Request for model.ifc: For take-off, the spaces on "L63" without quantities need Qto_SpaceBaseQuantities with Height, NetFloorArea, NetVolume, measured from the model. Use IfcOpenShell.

First a look at what the model holds.

```python
import ifcopenshell
import ifcopenshell.util.element
import ifcopenshell.util.unit

model = ifcopenshell.open("model.ifc")
print(model.schema)
for unit_type in ("LENGTHUNIT", "AREAUNIT", "VOLUMEUNIT"):
    print(unit_type, ifcopenshell.util.unit.calculate_unit_scale(model, unit_type))
storey = next(s for s in model.by_type("IfcBuildingStorey") if s.Name == "L63")
spaces = [e for e in ifcopenshell.util.element.get_decomposition(storey) if e.is_a("IfcSpace")]
for e in sorted(spaces, key=lambda e: e.id()):
    print(e.id(), e.is_a(), e.Name, list(ifcopenshell.util.element.get_psets(e, qtos_only=True)), sep=" | ")
```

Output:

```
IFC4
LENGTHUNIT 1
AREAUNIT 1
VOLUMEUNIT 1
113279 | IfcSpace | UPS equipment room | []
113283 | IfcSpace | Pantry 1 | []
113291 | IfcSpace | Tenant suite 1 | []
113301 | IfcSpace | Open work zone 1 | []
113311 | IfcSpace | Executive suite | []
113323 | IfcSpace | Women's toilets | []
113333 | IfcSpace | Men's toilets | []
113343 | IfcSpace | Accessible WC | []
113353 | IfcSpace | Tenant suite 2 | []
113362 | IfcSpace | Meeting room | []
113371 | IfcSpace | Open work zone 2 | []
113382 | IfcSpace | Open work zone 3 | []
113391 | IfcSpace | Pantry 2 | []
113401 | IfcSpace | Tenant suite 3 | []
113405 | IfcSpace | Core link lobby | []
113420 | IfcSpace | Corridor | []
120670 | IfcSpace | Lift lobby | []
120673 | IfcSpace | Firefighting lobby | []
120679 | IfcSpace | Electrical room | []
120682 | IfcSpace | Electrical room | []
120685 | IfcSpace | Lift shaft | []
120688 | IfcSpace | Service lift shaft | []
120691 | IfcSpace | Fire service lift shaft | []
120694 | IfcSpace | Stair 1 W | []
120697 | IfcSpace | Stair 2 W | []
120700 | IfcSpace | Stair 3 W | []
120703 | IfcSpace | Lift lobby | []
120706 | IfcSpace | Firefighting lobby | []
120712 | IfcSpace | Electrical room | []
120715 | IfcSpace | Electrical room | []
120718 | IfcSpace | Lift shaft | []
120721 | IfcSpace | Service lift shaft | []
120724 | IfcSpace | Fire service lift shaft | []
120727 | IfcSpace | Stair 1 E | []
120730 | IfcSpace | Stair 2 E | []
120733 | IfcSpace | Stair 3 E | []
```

```python
import ifcopenshell
import ifcopenshell.api.pset
import ifcopenshell.geom
import ifcopenshell.util.element
import ifcopenshell.util.shape
import ifcopenshell.util.unit

model = ifcopenshell.open("model.ifc")
unit_scale = ifcopenshell.util.unit.calculate_unit_scale(model)
area_scale = ifcopenshell.util.unit.calculate_unit_scale(model, "AREAUNIT")
volume_scale = ifcopenshell.util.unit.calculate_unit_scale(model, "VOLUMEUNIT")
settings = ifcopenshell.geom.settings()

storey = next(s for s in model.by_type("IfcBuildingStorey") if s.Name == "L63")
spaces = [e for e in ifcopenshell.util.element.get_decomposition(storey) if e.is_a("IfcSpace")]

for e in sorted(spaces, key=lambda e: e.id()):
    if ifcopenshell.util.element.get_psets(e, qtos_only=True, should_inherit=False):
        continue
    # Geometry comes back in metres, in the element's own axes.
    shape = ifcopenshell.geom.create_shape(settings, e)
    values = {
        "Height": ifcopenshell.util.shape.get_z(shape.geometry) / unit_scale,
        "NetFloorArea": ifcopenshell.util.shape.get_footprint_area(shape.geometry) / area_scale,
        "NetVolume": ifcopenshell.util.shape.get_volume(shape.geometry) / volume_scale,
    }
    qto = ifcopenshell.api.pset.add_qto(model, product=e, name="Qto_SpaceBaseQuantities")
    ifcopenshell.api.pset.edit_qto(model, qto=qto, properties=values)
    print(e.id(), {k: round(v, 3) for k, v in values.items()})

model.write("model_edited.ifc")
```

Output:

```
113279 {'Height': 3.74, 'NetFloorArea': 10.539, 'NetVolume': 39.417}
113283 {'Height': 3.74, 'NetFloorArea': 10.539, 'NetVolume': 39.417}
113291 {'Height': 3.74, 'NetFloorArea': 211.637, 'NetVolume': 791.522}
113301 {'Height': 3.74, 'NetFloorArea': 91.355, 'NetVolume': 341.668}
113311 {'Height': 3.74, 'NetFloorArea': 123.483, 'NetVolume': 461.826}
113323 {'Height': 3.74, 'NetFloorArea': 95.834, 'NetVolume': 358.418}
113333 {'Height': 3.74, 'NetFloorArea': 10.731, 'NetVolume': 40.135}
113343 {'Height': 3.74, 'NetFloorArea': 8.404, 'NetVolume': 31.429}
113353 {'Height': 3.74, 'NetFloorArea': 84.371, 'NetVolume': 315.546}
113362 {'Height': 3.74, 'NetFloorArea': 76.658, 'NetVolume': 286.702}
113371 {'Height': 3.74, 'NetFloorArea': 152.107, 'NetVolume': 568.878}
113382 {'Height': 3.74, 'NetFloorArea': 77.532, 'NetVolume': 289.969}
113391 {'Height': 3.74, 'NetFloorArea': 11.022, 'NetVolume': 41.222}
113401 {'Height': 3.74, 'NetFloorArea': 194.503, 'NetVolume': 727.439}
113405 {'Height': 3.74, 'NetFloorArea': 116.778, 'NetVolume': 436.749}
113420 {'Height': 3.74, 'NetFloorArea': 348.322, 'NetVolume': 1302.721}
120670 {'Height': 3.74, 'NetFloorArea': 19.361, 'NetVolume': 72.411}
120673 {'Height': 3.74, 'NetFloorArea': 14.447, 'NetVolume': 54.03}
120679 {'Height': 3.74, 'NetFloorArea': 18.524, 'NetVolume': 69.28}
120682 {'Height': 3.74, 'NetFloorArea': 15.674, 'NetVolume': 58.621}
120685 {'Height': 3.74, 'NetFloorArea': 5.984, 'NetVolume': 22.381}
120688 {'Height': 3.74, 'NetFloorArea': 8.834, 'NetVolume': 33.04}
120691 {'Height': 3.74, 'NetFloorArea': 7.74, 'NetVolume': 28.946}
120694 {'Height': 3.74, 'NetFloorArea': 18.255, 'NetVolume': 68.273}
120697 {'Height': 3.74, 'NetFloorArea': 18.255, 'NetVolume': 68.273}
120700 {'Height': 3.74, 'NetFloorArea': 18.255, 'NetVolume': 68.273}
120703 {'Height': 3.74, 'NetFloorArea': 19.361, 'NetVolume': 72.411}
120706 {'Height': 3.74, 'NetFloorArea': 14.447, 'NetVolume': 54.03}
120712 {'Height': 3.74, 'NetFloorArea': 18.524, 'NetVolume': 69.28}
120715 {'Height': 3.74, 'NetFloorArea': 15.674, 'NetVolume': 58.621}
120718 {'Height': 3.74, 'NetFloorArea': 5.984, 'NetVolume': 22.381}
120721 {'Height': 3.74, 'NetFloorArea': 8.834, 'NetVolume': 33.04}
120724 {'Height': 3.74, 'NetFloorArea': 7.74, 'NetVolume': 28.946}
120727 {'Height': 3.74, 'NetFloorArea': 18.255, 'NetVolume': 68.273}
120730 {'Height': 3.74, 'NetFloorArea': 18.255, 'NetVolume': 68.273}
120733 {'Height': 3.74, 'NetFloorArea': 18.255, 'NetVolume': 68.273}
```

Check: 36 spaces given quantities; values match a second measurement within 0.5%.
